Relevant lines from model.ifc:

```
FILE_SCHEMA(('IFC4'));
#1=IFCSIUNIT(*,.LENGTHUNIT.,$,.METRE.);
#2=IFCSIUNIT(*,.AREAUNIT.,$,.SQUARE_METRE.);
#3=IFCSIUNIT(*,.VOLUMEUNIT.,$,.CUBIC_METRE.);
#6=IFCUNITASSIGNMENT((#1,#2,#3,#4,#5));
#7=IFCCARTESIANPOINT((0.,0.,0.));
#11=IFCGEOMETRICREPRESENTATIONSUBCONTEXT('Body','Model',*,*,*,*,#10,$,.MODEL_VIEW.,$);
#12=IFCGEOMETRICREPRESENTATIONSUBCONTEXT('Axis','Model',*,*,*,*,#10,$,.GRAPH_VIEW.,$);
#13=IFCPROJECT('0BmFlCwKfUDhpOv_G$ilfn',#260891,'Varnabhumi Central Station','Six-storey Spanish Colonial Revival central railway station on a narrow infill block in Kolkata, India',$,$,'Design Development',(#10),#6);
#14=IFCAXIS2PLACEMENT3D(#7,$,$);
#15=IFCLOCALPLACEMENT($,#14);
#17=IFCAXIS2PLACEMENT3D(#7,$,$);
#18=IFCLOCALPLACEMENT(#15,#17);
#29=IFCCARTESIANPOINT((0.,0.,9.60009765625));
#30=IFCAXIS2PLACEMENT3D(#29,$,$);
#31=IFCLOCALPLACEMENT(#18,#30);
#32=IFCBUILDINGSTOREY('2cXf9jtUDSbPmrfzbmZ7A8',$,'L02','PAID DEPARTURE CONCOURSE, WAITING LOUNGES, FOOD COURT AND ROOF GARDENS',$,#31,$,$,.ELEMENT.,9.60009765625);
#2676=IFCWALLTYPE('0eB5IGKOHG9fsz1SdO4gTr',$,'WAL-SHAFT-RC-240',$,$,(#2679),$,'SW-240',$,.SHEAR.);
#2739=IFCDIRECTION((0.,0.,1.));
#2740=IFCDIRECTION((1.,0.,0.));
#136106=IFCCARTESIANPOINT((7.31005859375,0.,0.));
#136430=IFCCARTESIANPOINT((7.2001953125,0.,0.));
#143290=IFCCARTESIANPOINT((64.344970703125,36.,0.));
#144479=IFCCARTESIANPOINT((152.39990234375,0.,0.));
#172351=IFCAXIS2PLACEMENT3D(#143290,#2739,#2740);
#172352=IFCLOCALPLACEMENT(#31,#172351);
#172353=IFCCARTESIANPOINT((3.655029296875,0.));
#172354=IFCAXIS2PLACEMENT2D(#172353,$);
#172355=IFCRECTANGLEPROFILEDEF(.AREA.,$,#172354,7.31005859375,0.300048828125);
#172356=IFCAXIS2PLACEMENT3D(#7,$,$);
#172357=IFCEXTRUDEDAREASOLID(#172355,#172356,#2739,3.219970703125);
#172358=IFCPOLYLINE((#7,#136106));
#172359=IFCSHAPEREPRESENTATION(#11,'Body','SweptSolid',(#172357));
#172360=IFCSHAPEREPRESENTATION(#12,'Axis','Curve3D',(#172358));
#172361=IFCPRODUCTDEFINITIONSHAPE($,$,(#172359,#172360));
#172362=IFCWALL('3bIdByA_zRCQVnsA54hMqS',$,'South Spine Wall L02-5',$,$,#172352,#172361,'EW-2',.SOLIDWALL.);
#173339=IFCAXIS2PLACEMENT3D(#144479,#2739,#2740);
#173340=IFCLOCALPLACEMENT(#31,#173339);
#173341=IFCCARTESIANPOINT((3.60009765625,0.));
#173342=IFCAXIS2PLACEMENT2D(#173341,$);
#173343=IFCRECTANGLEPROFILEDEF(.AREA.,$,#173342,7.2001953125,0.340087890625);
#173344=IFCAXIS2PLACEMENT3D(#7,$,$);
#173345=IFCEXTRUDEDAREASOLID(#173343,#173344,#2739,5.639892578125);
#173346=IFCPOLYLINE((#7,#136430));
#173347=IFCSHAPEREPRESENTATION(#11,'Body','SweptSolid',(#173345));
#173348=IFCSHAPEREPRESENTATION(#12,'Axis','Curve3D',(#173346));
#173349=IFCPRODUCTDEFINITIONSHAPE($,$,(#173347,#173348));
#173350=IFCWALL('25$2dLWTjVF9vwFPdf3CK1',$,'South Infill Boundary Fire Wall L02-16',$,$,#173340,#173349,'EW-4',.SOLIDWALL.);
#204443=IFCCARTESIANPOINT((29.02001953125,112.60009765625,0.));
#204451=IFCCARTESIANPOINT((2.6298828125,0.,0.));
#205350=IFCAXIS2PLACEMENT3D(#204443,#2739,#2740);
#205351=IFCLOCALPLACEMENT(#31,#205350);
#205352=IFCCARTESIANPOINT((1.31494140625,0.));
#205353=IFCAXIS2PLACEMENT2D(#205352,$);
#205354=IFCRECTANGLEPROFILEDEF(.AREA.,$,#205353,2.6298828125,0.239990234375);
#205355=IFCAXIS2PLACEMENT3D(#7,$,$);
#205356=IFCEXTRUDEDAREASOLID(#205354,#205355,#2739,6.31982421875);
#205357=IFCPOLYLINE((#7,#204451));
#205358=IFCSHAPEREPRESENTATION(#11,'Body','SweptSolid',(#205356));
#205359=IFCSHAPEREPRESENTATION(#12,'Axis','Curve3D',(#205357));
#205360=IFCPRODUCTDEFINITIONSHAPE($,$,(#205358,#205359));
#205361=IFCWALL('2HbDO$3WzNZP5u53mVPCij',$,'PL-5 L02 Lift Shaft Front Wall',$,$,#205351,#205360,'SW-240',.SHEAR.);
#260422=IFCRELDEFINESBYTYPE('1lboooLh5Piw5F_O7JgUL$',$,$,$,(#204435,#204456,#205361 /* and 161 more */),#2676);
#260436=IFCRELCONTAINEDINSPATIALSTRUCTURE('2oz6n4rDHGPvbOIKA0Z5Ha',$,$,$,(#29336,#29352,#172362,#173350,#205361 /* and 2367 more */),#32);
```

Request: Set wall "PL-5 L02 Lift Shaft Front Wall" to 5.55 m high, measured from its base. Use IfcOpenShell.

```python
import ifcopenshell
import ifcopenshell.geom
import ifcopenshell.util.representation
import ifcopenshell.util.shape

model = ifcopenshell.open("model.ifc")
settings = ifcopenshell.geom.settings()


def volume(element):
    """Net volume in cubic metres, openings subtracted."""
    shape = ifcopenshell.geom.create_shape(settings, element)
    return ifcopenshell.util.shape.get_volume(shape.geometry)


wall = model.by_guid("2HbDO$3WzNZP5u53mVPCij")
before = volume(wall)

body = ifcopenshell.util.representation.get_representation(wall, "Model", "Body")
solid = body.Items[0]
old_height = solid.Depth
solid.Depth = 5.55
after = volume(wall)

print(f"height {old_height:g} -> {solid.Depth:g}, volume {before:.3f} -> {after:.3f} m3")

model.write("model-out.ifc")
```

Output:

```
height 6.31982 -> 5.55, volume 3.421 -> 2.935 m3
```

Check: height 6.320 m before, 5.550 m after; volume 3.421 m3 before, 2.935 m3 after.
